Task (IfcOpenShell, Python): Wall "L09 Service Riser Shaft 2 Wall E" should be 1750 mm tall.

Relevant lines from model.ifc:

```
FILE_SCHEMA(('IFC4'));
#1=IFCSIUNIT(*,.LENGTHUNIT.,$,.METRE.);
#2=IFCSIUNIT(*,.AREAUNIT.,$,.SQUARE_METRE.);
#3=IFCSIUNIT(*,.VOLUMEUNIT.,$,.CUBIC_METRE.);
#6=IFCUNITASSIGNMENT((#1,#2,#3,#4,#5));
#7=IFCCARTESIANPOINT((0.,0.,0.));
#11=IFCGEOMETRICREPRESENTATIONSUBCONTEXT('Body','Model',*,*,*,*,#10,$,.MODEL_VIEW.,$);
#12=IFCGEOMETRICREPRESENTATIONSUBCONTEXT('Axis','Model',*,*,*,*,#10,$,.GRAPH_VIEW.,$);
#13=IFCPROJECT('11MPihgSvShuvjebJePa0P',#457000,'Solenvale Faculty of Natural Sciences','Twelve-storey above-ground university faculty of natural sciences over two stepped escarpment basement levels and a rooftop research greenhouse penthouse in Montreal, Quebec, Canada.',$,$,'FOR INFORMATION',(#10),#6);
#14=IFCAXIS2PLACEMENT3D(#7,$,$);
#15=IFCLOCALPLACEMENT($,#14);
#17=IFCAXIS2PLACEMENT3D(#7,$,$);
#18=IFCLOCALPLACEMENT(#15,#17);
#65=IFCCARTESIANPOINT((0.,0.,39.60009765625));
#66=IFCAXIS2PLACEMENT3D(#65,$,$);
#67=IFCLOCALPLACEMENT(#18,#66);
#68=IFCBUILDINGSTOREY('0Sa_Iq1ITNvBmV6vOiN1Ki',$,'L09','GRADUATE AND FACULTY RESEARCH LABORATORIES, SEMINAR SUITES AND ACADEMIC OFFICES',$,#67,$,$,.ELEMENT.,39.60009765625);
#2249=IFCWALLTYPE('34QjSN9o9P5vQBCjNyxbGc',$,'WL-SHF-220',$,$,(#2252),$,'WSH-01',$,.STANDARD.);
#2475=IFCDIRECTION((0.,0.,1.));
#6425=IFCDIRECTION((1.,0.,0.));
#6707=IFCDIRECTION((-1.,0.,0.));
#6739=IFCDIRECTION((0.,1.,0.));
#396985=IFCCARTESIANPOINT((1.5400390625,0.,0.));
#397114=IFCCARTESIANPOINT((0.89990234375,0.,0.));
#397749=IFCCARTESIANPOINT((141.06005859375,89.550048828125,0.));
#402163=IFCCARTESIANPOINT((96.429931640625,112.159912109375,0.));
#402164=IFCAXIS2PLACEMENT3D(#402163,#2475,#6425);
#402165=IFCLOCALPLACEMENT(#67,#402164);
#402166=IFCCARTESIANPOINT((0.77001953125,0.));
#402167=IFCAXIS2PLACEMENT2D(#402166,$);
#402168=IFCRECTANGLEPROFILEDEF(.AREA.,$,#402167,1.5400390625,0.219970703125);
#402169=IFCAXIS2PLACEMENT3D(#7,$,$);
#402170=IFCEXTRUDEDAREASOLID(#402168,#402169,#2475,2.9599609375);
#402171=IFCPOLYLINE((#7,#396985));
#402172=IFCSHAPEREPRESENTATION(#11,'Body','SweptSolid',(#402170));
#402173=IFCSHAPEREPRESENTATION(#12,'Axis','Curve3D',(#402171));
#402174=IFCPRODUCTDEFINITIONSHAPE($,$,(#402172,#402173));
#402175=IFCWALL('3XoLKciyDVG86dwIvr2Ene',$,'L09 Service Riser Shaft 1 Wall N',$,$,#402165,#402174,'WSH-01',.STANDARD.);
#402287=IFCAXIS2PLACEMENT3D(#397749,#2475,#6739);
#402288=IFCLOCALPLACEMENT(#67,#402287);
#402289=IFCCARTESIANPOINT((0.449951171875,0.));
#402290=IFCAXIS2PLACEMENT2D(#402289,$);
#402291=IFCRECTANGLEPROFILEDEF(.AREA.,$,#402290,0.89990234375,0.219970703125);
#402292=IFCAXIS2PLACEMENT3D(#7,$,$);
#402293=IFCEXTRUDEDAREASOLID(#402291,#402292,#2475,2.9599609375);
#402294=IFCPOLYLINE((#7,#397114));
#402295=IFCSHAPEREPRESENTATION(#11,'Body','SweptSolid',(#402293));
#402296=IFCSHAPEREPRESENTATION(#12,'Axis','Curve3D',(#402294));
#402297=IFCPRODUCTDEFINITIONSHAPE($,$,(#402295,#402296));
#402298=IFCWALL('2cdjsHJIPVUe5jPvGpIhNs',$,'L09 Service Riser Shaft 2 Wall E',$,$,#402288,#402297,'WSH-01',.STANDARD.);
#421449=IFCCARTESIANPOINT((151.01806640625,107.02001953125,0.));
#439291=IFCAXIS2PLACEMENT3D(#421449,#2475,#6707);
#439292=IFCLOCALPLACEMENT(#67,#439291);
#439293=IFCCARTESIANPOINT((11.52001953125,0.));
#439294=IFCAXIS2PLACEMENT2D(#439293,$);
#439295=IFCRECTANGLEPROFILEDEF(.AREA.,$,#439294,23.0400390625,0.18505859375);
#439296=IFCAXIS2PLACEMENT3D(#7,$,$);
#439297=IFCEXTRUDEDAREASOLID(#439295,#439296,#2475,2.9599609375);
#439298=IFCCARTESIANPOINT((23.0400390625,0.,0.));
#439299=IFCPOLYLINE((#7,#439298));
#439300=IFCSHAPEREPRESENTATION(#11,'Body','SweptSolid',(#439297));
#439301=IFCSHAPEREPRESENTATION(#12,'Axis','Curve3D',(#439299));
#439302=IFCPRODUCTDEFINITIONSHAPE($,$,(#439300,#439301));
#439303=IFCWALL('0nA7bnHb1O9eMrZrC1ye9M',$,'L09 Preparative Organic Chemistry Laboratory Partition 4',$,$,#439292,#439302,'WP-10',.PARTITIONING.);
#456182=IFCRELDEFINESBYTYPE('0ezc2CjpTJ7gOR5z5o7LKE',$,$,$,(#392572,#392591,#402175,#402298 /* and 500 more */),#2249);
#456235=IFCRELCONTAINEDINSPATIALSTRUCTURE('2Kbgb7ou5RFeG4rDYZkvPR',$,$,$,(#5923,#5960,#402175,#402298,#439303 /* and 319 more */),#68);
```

```python
import ifcopenshell
import ifcopenshell.geom
import ifcopenshell.util.representation
import ifcopenshell.util.shape
import ifcopenshell.util.unit

model = ifcopenshell.open("model.ifc")
unit_scale = ifcopenshell.util.unit.calculate_unit_scale(model)
settings = ifcopenshell.geom.settings()


def volume(element):
    """Net volume in cubic metres, openings subtracted."""
    shape = ifcopenshell.geom.create_shape(settings, element)
    return ifcopenshell.util.shape.get_volume(shape.geometry)


wall = model.by_id(402298)
before = volume(wall)

body = ifcopenshell.util.representation.get_representation(wall, "Model", "Body")
solid = body.Items[0]
old_height = solid.Depth
solid.Depth = 1.75 / unit_scale
after = volume(wall)

print(f"height {old_height:g} -> {solid.Depth:g}, volume {before:.3f} -> {after:.3f} m3")

model.write("model_v2.ifc")
```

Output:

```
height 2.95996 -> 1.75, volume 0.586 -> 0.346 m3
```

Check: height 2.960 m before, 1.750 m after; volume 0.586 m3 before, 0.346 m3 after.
